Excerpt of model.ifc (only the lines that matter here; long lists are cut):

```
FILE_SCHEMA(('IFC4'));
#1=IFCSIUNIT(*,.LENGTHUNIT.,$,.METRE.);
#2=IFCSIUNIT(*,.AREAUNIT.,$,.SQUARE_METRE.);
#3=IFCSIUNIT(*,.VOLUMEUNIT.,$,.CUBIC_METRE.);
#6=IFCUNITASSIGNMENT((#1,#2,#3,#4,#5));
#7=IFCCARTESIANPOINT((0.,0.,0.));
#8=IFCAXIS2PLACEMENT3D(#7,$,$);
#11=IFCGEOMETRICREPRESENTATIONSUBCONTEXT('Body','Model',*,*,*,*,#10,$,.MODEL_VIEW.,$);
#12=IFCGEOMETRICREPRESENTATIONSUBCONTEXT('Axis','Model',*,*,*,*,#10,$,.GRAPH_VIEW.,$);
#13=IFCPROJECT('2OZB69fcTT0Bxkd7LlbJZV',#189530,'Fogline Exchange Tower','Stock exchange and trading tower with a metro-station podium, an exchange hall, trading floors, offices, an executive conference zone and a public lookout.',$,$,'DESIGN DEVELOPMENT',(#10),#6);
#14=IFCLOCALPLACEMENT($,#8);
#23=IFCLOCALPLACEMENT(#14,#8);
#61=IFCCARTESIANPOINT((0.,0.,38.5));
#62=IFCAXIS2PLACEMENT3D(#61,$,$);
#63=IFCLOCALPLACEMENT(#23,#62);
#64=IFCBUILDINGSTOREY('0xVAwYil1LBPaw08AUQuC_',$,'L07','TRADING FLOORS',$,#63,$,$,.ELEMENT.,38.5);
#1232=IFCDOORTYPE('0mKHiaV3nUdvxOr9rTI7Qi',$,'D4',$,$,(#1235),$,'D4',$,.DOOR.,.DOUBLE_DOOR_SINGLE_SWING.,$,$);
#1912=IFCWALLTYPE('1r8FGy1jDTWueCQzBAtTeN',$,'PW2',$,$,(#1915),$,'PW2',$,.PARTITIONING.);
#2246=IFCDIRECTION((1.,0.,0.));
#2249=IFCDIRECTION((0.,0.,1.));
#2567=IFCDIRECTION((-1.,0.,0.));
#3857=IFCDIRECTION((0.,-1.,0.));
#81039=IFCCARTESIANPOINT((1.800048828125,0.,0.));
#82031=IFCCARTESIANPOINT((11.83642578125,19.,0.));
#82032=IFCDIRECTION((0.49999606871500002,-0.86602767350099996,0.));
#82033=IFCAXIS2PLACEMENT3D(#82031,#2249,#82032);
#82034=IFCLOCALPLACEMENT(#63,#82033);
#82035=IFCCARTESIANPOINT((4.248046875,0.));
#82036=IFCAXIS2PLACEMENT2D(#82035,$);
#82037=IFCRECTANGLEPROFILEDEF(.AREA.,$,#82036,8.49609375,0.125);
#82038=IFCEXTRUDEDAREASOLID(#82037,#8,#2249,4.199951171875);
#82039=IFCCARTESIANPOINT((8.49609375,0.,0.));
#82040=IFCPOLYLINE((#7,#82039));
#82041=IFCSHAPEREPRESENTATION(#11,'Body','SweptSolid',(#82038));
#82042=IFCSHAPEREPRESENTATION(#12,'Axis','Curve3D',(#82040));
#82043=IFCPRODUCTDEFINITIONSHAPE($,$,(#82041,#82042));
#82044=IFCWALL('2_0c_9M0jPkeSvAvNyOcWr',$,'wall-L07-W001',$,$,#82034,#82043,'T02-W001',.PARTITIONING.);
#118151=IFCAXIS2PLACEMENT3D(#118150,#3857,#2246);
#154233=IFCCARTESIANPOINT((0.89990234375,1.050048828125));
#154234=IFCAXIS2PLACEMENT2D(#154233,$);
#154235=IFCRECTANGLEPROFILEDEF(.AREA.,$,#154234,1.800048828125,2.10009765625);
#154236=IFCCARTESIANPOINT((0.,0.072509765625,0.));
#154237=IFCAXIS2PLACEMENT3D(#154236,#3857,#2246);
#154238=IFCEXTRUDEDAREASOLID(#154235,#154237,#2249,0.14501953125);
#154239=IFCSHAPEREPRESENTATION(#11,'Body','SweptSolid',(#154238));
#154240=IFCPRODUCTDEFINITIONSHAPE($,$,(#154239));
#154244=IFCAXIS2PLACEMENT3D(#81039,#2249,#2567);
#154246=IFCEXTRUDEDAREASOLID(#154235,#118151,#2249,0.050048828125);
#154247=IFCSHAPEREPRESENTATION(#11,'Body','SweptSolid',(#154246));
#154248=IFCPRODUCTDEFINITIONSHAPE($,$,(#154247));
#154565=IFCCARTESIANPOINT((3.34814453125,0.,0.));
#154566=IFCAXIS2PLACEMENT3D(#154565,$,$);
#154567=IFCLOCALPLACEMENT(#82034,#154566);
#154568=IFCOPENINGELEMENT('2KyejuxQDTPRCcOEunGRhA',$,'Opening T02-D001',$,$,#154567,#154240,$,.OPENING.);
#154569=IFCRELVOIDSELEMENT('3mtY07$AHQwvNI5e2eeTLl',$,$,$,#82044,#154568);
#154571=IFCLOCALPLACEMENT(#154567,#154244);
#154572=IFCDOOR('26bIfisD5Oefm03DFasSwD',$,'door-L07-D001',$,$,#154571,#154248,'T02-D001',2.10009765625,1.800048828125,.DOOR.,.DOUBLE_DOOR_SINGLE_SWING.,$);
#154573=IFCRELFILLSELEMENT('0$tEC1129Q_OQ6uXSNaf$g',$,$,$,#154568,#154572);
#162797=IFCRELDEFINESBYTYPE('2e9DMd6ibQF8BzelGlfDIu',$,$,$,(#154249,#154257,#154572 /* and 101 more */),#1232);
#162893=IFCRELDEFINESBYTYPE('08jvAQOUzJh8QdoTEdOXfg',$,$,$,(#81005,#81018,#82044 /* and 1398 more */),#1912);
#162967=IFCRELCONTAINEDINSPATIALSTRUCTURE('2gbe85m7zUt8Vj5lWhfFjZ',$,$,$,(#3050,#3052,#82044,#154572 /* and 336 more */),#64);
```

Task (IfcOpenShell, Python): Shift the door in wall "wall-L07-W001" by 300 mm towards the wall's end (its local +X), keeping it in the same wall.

```python
import ifcopenshell
import ifcopenshell.api.geometry
import ifcopenshell.util.placement
import ifcopenshell.util.unit

model = ifcopenshell.open("model.ifc")
unit_scale = ifcopenshell.util.unit.calculate_unit_scale(model)

door = model.by_guid("26bIfisD5Oefm03DFasSwD")
opening = door.FillsVoids[0].RelatingOpeningElement
wall = opening.VoidsElements[0].RelatingBuildingElement

wall_matrix = ifcopenshell.util.placement.get_local_placement(wall.ObjectPlacement)
shift = wall_matrix[:3, 0] * 0.3 / unit_scale
before = ifcopenshell.util.placement.get_local_placement(door.ObjectPlacement)[:3, 3].copy()

# The door is placed relative to its opening, so it follows when the opening moves.
matrix = ifcopenshell.util.placement.get_local_placement(opening.ObjectPlacement)
matrix[:3, 3] += shift
ifcopenshell.api.geometry.edit_object_placement(
    model, product=opening, matrix=matrix, is_si=False, should_transform_children=True
)

after = ifcopenshell.util.placement.get_local_placement(door.ObjectPlacement)[:3, 3]
print("door moved by", (after - before).round(3) + 0.0)

model.write("model_rev.ifc")
```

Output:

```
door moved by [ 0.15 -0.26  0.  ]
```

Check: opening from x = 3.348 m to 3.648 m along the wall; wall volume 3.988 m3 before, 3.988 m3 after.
